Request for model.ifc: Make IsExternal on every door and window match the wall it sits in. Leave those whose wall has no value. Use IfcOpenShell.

First a look at what the model holds.

```python
import ifcopenshell
import ifcopenshell.util.element

model = ifcopenshell.open("model.ifc")
print(model.schema)
seen = {}
for e in model.by_type("IfcDoor") + model.by_type("IfcWindow"):
    if not e.FillsVoids:
        continue
    host = e.FillsVoids[0].RelatingOpeningElement.VoidsElements[0].RelatingBuildingElement
    own = ifcopenshell.util.element.get_pset(e, f"Pset_{e.is_a()[3:].removesuffix('StandardCase')}Common", "IsExternal")
    wall = ifcopenshell.util.element.get_pset(host, "Pset_WallCommon", "IsExternal")
    seen[e.is_a(), own, wall] = seen.get((e.is_a(), own, wall), 0) + 1
for (cls, own, wall), count in sorted(seen.items(), key=str):
    print(count, cls, "IsExternal:", own, "| host wall:", wall)
```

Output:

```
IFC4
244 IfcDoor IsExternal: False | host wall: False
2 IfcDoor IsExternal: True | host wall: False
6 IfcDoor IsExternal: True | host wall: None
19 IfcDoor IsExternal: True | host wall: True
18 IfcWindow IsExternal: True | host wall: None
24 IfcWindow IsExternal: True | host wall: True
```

```python
import ifcopenshell
import ifcopenshell.api.pset
import ifcopenshell.util.element

model = ifcopenshell.open("model.ifc")

count = 0
for ifc_class, pset_name in (("IfcDoor", "Pset_DoorCommon"), ("IfcWindow", "Pset_WindowCommon")):
    for e in model.by_type(ifc_class):
        if not e.FillsVoids:
            continue
        host = e.FillsVoids[0].RelatingOpeningElement.VoidsElements[0].RelatingBuildingElement
        external = ifcopenshell.util.element.get_pset(host, "Pset_WallCommon", "IsExternal")
        if external is None or ifcopenshell.util.element.get_pset(e, pset_name, "IsExternal") == external:
            continue
        pset = ifcopenshell.api.pset.add_pset(model, product=e, name=pset_name)
        ifcopenshell.api.pset.edit_pset(model, pset=pset, properties={"IsExternal": external})
        count += 1

print(count, "updated")

model.write("model_rev.ifc")
```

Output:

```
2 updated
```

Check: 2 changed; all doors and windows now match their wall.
